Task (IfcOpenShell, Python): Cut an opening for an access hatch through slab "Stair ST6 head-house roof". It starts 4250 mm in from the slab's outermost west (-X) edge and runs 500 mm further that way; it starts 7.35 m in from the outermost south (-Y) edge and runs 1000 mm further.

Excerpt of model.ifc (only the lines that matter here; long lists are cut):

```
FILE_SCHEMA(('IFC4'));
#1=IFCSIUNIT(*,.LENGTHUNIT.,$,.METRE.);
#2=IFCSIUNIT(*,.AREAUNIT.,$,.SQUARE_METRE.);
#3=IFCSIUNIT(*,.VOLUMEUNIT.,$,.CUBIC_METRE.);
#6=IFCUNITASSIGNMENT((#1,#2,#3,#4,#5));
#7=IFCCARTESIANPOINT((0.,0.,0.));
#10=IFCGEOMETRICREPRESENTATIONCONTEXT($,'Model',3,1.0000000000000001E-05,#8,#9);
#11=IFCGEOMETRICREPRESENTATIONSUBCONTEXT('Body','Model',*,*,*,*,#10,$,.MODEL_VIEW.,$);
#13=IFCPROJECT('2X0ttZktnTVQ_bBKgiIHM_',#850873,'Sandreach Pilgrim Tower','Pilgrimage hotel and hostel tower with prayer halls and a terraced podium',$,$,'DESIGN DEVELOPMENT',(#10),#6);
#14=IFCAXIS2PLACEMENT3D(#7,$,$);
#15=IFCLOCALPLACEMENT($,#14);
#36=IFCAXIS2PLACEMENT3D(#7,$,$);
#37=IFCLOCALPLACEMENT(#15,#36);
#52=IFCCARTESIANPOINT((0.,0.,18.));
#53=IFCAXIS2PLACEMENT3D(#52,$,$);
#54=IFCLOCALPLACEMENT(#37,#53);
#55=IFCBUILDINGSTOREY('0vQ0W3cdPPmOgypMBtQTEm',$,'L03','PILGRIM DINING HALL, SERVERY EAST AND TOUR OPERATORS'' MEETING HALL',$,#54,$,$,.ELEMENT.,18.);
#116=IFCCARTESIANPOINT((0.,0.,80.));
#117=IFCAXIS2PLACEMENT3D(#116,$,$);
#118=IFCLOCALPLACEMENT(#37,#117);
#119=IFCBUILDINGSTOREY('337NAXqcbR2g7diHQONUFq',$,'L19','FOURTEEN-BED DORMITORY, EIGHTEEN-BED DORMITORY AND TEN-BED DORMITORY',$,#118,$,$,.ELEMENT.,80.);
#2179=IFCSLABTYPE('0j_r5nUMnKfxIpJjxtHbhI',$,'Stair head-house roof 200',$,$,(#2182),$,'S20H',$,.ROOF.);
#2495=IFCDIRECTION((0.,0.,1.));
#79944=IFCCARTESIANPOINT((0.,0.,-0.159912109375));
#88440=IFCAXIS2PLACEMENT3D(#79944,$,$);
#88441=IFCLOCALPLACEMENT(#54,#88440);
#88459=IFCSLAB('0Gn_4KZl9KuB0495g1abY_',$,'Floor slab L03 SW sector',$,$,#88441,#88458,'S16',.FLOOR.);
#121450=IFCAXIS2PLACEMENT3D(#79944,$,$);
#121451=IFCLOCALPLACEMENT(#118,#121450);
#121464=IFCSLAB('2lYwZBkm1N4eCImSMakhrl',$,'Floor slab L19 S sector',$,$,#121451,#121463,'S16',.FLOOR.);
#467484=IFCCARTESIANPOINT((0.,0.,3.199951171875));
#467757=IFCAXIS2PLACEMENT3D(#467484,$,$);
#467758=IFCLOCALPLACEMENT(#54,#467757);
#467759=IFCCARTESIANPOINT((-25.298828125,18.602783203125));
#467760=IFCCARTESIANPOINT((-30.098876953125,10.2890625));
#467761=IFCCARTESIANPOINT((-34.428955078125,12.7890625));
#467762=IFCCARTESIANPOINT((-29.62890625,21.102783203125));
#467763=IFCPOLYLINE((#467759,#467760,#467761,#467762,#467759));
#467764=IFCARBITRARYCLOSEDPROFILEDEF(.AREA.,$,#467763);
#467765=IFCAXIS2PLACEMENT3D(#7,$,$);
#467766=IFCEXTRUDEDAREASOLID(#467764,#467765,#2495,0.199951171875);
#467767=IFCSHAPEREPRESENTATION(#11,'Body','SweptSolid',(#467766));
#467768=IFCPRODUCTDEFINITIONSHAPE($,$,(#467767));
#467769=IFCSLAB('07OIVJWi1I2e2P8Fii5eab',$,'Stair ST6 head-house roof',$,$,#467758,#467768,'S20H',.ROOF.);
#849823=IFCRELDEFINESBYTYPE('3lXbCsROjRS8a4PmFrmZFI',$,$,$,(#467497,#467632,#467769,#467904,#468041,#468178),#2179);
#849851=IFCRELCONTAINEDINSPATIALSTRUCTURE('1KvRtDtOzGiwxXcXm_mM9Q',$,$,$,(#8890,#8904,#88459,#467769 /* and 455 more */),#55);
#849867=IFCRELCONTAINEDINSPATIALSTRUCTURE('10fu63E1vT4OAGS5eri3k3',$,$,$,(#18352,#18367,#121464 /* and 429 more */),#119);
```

```python
import numpy as np
import ifcopenshell
import ifcopenshell.api.feature
import ifcopenshell.api.geometry
import ifcopenshell.api.root
import ifcopenshell.geom
import ifcopenshell.util.placement
import ifcopenshell.util.representation
import ifcopenshell.util.shape
import ifcopenshell.util.unit

model = ifcopenshell.open("model.ifc")
unit_scale = ifcopenshell.util.unit.calculate_unit_scale(model)
settings = ifcopenshell.geom.settings()


def volume(element):
    """Net volume in cubic metres, openings subtracted."""
    shape = ifcopenshell.geom.create_shape(settings, element)
    return ifcopenshell.util.shape.get_volume(shape.geometry)


slab = model.by_guid("07OIVJWi1I2e2P8Fii5eab")
before = volume(slab)

# Extent in the slab's own axes, in metres. The edges named are its -X and -Y sides.
slab_shape = ifcopenshell.geom.create_shape(settings, slab)
vertices = ifcopenshell.util.shape.get_vertices(slab_shape.geometry)
x_min, y_min, bottom = vertices.min(axis=0)
top = vertices[:, 2].max()

opening = ifcopenshell.api.root.create_entity(model, ifc_class="IfcOpeningElement", name="Access hatch opening", predefined_type="OPENING")
context = ifcopenshell.util.representation.get_context(model, "Model", "Body", "MODEL_VIEW")
width, depth = 0.5, 1
outline = [(0.0, 0.0), (width, 0.0), (width, depth), (0.0, depth), (0.0, 0.0)]
# Overshoot both faces by 50 mm so the cut is clean.
shape = ifcopenshell.api.geometry.add_slab_representation(
    model, context=context, depth=top - bottom + 0.1, polyline=outline
)
ifcopenshell.api.geometry.assign_representation(model, product=opening, representation=shape)

matrix = ifcopenshell.util.placement.get_local_placement(slab.ObjectPlacement)
matrix[:, 3] = matrix @ np.append(np.array([x_min + 4.25, y_min + 7.35, bottom - 0.05]) / unit_scale, 1.0)
ifcopenshell.api.geometry.edit_object_placement(model, product=opening, matrix=matrix, is_si=False)
ifcopenshell.api.feature.add_feature(model, feature=opening, element=slab)

after = volume(slab)

print(f"slab volume {before:.3f} -> {after:.3f} m3")

model.write("model_rev.ifc")
```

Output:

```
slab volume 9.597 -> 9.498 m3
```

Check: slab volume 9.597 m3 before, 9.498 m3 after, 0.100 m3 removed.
